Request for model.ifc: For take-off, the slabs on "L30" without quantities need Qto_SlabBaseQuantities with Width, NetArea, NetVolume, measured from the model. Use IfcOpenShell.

First a look at what the model holds.

```python
import ifcopenshell
import ifcopenshell.util.element
import ifcopenshell.util.unit

model = ifcopenshell.open("model.ifc")
print(model.schema)
for unit_type in ("LENGTHUNIT", "AREAUNIT", "VOLUMEUNIT"):
    print(unit_type, ifcopenshell.util.unit.calculate_unit_scale(model, unit_type))
storey = next(s for s in model.by_type("IfcBuildingStorey") if s.Name == "L30")
slabs = [e for e in ifcopenshell.util.element.get_decomposition(storey) if e.is_a("IfcSlab")]
for e in sorted(slabs, key=lambda e: e.id()):
    print(e.id(), e.is_a(), e.Name, list(ifcopenshell.util.element.get_psets(e, qtos_only=True)), sep=" | ")
```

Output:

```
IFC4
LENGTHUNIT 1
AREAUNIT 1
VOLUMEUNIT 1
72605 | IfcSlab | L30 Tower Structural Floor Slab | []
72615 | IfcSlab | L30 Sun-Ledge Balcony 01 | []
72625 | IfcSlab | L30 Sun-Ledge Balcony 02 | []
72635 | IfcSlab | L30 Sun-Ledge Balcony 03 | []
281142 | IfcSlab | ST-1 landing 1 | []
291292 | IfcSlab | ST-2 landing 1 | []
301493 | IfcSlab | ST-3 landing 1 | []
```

```python
import ifcopenshell
import ifcopenshell.api.pset
import ifcopenshell.geom
import ifcopenshell.util.element
import ifcopenshell.util.shape
import ifcopenshell.util.unit

model = ifcopenshell.open("model.ifc")
unit_scale = ifcopenshell.util.unit.calculate_unit_scale(model)
area_scale = ifcopenshell.util.unit.calculate_unit_scale(model, "AREAUNIT")
volume_scale = ifcopenshell.util.unit.calculate_unit_scale(model, "VOLUMEUNIT")
settings = ifcopenshell.geom.settings()

storey = next(s for s in model.by_type("IfcBuildingStorey") if s.Name == "L30")
slabs = [e for e in ifcopenshell.util.element.get_decomposition(storey) if e.is_a("IfcSlab")]

for e in sorted(slabs, key=lambda e: e.id()):
    if ifcopenshell.util.element.get_psets(e, qtos_only=True, should_inherit=False):
        continue
    # Geometry comes back in metres, in the element's own axes.
    shape = ifcopenshell.geom.create_shape(settings, e)
    values = {
        "Width": ifcopenshell.util.shape.get_z(shape.geometry) / unit_scale,
        "NetArea": ifcopenshell.util.shape.get_footprint_area(shape.geometry) / area_scale,
        "NetVolume": ifcopenshell.util.shape.get_volume(shape.geometry) / volume_scale,
    }
    qto = ifcopenshell.api.pset.add_qto(model, product=e, name="Qto_SlabBaseQuantities")
    ifcopenshell.api.pset.edit_qto(model, qto=qto, properties=values)
    print(e.id(), {k: round(v, 3) for k, v in values.items()})

model.write("model-out.ifc")
```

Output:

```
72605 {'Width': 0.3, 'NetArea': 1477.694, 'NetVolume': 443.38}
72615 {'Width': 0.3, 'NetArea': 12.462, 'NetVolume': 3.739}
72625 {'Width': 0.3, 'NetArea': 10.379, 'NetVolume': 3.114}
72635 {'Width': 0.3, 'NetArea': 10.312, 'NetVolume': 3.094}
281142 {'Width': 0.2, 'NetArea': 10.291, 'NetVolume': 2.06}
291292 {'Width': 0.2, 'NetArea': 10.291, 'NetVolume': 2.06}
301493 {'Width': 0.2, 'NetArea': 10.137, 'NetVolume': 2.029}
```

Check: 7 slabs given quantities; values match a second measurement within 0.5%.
